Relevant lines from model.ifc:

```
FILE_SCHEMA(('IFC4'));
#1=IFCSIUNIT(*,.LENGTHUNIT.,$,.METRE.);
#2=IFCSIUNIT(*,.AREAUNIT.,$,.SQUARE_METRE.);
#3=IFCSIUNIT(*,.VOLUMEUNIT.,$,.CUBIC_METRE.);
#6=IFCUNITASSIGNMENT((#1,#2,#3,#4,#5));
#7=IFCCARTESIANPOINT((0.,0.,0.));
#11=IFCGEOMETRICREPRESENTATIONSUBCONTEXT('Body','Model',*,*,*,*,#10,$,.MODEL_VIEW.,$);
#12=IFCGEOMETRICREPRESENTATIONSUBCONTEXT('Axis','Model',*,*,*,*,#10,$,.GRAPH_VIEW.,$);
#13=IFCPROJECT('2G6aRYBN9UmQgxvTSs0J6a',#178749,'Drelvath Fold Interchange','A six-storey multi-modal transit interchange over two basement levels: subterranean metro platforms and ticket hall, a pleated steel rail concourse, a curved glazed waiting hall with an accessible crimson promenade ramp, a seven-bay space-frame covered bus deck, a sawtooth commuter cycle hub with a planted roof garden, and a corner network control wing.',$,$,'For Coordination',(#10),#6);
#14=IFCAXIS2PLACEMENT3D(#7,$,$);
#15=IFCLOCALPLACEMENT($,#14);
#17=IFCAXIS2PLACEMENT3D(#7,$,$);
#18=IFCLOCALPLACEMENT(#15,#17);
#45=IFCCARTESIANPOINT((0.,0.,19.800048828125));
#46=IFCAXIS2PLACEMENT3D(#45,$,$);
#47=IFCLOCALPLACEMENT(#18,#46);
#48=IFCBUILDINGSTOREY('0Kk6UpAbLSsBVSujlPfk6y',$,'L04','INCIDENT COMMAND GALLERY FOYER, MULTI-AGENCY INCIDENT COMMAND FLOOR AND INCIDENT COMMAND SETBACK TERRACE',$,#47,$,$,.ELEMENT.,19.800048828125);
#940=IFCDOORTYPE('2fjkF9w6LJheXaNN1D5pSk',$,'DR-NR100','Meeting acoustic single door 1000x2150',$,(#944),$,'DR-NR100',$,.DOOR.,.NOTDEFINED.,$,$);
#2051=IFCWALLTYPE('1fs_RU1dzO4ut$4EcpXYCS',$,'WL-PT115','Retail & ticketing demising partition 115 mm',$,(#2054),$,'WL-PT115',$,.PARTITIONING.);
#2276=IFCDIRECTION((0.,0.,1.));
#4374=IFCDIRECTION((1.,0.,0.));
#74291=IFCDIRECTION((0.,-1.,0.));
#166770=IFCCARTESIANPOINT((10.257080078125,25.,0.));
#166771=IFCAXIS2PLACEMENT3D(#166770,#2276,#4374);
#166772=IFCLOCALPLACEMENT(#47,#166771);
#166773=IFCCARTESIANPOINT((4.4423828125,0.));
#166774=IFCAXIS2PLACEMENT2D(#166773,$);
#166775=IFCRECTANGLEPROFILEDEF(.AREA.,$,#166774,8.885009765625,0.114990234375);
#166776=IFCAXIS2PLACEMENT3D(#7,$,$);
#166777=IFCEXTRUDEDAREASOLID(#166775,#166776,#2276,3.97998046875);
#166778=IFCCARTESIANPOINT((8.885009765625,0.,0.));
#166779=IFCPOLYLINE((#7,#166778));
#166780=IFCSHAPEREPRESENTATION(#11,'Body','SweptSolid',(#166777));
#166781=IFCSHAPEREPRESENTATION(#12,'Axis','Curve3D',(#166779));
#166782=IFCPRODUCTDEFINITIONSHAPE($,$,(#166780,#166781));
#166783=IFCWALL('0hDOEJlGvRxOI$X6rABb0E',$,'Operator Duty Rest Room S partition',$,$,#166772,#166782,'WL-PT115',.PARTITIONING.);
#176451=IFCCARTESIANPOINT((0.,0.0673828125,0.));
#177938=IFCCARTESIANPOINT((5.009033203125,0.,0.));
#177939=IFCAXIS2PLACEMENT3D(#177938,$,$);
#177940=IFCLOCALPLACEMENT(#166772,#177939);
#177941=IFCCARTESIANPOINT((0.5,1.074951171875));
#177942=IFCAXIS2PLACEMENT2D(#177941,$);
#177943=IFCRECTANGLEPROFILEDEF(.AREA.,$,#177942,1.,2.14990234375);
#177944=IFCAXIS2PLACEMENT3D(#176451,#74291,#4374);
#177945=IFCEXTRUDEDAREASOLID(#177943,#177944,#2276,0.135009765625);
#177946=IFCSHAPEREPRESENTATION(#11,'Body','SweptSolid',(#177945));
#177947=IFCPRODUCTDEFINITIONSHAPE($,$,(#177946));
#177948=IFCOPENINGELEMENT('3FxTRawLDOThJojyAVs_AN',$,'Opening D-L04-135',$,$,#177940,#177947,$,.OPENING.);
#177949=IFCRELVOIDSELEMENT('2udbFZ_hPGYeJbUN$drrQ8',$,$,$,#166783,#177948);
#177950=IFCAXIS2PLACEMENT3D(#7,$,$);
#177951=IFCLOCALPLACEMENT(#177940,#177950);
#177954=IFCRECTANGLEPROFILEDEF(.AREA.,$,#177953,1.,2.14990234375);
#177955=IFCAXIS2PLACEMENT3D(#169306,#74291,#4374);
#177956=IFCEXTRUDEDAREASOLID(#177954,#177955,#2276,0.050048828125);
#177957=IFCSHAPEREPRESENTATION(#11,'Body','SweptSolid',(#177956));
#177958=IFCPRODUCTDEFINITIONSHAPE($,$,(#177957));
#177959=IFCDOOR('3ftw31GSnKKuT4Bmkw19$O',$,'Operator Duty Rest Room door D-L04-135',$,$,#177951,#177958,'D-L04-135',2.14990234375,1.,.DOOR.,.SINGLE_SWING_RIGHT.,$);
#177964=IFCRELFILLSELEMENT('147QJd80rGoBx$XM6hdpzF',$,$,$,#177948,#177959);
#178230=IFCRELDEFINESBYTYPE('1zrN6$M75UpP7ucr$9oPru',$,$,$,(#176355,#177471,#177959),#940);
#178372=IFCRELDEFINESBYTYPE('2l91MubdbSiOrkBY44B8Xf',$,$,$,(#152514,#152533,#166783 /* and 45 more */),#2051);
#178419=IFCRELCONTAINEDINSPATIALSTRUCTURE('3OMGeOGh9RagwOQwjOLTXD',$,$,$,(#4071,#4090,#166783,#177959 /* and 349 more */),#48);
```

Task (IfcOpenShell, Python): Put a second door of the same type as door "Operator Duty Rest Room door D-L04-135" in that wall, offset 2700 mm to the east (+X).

```python
import ifcopenshell
import ifcopenshell.api.feature
import ifcopenshell.api.geometry
import ifcopenshell.api.root
import ifcopenshell.geom
import ifcopenshell.util.element
import ifcopenshell.util.placement
import ifcopenshell.util.shape
import ifcopenshell.util.unit

model = ifcopenshell.open("model.ifc")
unit_scale = ifcopenshell.util.unit.calculate_unit_scale(model)
settings = ifcopenshell.geom.settings()


def volume(element):
    """Net volume in cubic metres, openings subtracted."""
    shape = ifcopenshell.geom.create_shape(settings, element)
    return ifcopenshell.util.shape.get_volume(shape.geometry)


door = model.by_guid("3ftw31GSnKKuT4Bmkw19$O")
opening = door.FillsVoids[0].RelatingOpeningElement
wall = opening.VoidsElements[0].RelatingBuildingElement
before = volume(wall)
shift = ifcopenshell.util.placement.get_local_placement(wall.ObjectPlacement)[:3, 0] * 2.7 / unit_scale

# copy_class copies the void relationship, type, container and properties, but no geometry.
new_opening = ifcopenshell.api.root.copy_class(model, product=opening)
new_opening.Representation = ifcopenshell.util.element.copy_deep(
    model, opening.Representation, exclude=["IfcGeometricRepresentationContext", "IfcRepresentationMap"]
)
new_door = ifcopenshell.api.root.copy_class(model, product=door)
new_door.Representation = ifcopenshell.util.element.copy_deep(
    model, door.Representation, exclude=["IfcGeometricRepresentationContext", "IfcRepresentationMap"]
)
new_door.Tag = None
ifcopenshell.api.feature.add_filling(model, opening=new_opening, element=new_door)

for old, new in ((opening, new_opening), (door, new_door)):
    matrix = ifcopenshell.util.placement.get_local_placement(old.ObjectPlacement)
    matrix[:3, 3] += shift
    ifcopenshell.api.geometry.edit_object_placement(model, product=new, matrix=matrix, is_si=False)

after = volume(wall)

print(f"wall volume {before:.3f} -> {after:.3f} m3")

model.write("model_v2.ifc")
```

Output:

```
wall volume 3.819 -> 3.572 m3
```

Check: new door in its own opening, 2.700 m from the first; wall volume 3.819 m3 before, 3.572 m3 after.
